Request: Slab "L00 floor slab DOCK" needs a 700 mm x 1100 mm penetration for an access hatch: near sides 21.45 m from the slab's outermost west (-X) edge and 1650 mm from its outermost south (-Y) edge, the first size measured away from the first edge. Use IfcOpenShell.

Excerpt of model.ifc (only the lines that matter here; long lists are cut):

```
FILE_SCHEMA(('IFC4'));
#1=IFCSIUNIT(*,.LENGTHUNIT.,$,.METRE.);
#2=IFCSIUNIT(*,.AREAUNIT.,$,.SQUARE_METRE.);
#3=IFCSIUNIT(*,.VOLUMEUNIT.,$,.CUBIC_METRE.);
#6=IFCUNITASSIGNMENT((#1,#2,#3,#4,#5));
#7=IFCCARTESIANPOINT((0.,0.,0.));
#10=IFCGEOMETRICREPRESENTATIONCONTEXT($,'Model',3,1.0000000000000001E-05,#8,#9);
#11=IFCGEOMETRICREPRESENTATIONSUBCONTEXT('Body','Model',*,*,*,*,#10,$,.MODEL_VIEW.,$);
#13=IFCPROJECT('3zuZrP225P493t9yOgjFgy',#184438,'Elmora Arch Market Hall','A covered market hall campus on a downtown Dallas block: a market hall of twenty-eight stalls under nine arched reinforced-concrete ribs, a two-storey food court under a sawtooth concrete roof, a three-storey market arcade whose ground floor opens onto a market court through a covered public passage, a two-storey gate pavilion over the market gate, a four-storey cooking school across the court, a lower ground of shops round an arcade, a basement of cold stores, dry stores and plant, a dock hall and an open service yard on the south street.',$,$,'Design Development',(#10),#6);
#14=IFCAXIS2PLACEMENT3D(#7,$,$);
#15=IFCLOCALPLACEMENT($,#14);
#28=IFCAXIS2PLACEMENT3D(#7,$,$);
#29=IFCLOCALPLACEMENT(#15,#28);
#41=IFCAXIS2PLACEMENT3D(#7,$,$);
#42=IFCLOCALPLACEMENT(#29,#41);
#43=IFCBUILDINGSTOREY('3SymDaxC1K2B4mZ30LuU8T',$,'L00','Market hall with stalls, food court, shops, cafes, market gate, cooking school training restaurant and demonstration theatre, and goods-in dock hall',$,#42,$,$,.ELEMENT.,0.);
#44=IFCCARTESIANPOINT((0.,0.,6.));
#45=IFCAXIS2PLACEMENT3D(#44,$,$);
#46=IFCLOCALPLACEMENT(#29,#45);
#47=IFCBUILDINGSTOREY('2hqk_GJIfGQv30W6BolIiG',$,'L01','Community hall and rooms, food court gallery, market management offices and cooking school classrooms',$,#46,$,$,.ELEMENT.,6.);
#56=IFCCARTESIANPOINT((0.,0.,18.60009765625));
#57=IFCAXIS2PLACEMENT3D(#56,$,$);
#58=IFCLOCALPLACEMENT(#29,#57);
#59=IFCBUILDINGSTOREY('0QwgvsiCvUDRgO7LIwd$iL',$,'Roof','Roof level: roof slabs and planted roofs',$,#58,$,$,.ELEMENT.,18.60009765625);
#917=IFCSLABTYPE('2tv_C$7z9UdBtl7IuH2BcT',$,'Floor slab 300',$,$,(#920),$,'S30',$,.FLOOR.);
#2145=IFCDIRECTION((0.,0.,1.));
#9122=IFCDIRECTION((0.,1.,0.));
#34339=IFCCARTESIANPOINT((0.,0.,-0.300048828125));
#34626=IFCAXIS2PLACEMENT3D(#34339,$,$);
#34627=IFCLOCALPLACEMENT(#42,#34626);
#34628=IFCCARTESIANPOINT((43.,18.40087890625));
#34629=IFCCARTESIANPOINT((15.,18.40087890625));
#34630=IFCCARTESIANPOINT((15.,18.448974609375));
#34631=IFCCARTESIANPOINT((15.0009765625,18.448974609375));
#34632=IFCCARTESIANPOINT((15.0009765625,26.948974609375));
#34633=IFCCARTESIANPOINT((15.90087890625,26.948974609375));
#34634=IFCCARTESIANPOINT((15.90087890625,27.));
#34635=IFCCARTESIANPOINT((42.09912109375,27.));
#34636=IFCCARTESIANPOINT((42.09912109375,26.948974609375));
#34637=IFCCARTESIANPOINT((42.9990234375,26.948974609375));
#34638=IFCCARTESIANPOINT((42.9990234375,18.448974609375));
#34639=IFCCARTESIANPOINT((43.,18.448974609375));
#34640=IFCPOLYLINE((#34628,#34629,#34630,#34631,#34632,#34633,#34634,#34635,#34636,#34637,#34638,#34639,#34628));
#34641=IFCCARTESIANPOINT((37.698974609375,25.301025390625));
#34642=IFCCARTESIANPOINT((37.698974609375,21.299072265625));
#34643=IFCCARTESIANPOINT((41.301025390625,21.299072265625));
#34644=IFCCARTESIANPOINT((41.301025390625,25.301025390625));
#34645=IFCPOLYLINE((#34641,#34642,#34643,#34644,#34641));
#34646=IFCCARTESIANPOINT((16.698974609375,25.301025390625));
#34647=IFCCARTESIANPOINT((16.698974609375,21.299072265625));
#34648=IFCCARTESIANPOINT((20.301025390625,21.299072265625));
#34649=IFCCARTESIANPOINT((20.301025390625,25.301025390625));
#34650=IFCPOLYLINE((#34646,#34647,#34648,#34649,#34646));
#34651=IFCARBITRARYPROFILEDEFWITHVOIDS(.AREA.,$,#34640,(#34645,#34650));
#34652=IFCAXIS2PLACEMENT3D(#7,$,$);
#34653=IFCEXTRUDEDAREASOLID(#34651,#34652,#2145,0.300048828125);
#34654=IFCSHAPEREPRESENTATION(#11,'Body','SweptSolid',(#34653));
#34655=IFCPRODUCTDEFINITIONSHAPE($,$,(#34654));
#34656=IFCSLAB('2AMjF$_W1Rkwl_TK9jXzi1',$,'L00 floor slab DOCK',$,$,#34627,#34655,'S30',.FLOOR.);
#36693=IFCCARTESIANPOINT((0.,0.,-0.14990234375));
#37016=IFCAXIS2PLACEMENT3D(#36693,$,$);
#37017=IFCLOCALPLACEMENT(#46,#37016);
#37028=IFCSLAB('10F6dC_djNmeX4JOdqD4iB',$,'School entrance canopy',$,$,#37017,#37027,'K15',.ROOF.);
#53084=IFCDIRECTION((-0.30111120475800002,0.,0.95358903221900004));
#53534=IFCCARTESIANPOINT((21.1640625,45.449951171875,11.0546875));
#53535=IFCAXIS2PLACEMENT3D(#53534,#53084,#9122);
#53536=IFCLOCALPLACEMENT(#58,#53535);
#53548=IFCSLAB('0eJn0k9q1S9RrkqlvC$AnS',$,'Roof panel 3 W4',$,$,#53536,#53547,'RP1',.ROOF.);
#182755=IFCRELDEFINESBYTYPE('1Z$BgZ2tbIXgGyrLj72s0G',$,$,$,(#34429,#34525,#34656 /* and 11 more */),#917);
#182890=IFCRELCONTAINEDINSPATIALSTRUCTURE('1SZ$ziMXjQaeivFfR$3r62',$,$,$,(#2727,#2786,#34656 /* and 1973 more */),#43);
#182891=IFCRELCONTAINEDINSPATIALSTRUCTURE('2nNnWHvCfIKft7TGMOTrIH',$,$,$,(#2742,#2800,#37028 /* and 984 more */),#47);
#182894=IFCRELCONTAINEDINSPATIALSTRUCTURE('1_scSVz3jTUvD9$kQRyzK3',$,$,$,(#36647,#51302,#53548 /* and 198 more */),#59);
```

```python
import numpy as np
import ifcopenshell
import ifcopenshell.api.feature
import ifcopenshell.api.geometry
import ifcopenshell.api.root
import ifcopenshell.geom
import ifcopenshell.util.placement
import ifcopenshell.util.representation
import ifcopenshell.util.shape
import ifcopenshell.util.unit

model = ifcopenshell.open("model.ifc")
unit_scale = ifcopenshell.util.unit.calculate_unit_scale(model)
settings = ifcopenshell.geom.settings()


def volume(element):
    """Net volume in cubic metres, openings subtracted."""
    shape = ifcopenshell.geom.create_shape(settings, element)
    return ifcopenshell.util.shape.get_volume(shape.geometry)


slab = model.by_guid("2AMjF$_W1Rkwl_TK9jXzi1")
before = volume(slab)

# Extent in the slab's own axes, in metres. The edges named are its -X and -Y sides.
slab_shape = ifcopenshell.geom.create_shape(settings, slab)
vertices = ifcopenshell.util.shape.get_vertices(slab_shape.geometry)
x_min, y_min, bottom = vertices.min(axis=0)
top = vertices[:, 2].max()

opening = ifcopenshell.api.root.create_entity(model, ifc_class="IfcOpeningElement", name="Access hatch opening", predefined_type="OPENING")
context = ifcopenshell.util.representation.get_context(model, "Model", "Body", "MODEL_VIEW")
width, depth = 0.7, 1.1
outline = [(0.0, 0.0), (width, 0.0), (width, depth), (0.0, depth), (0.0, 0.0)]
# Overshoot both faces by 50 mm so the cut is clean.
shape = ifcopenshell.api.geometry.add_slab_representation(
    model, context=context, depth=top - bottom + 0.1, polyline=outline
)
ifcopenshell.api.geometry.assign_representation(model, product=opening, representation=shape)

matrix = ifcopenshell.util.placement.get_local_placement(slab.ObjectPlacement)
matrix[:, 3] = matrix @ np.append(np.array([x_min + 21.45, y_min + 1.65, bottom - 0.05]) / unit_scale, 1.0)
ifcopenshell.api.geometry.edit_object_placement(model, product=opening, matrix=matrix, is_si=False)
ifcopenshell.api.feature.add_feature(model, feature=opening, element=slab)

after = volume(slab)

print(f"slab volume {before:.3f} -> {after:.3f} m3")

model.write("model_rev.ifc")
```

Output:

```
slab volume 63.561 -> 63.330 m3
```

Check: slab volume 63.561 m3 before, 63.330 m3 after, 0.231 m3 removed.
